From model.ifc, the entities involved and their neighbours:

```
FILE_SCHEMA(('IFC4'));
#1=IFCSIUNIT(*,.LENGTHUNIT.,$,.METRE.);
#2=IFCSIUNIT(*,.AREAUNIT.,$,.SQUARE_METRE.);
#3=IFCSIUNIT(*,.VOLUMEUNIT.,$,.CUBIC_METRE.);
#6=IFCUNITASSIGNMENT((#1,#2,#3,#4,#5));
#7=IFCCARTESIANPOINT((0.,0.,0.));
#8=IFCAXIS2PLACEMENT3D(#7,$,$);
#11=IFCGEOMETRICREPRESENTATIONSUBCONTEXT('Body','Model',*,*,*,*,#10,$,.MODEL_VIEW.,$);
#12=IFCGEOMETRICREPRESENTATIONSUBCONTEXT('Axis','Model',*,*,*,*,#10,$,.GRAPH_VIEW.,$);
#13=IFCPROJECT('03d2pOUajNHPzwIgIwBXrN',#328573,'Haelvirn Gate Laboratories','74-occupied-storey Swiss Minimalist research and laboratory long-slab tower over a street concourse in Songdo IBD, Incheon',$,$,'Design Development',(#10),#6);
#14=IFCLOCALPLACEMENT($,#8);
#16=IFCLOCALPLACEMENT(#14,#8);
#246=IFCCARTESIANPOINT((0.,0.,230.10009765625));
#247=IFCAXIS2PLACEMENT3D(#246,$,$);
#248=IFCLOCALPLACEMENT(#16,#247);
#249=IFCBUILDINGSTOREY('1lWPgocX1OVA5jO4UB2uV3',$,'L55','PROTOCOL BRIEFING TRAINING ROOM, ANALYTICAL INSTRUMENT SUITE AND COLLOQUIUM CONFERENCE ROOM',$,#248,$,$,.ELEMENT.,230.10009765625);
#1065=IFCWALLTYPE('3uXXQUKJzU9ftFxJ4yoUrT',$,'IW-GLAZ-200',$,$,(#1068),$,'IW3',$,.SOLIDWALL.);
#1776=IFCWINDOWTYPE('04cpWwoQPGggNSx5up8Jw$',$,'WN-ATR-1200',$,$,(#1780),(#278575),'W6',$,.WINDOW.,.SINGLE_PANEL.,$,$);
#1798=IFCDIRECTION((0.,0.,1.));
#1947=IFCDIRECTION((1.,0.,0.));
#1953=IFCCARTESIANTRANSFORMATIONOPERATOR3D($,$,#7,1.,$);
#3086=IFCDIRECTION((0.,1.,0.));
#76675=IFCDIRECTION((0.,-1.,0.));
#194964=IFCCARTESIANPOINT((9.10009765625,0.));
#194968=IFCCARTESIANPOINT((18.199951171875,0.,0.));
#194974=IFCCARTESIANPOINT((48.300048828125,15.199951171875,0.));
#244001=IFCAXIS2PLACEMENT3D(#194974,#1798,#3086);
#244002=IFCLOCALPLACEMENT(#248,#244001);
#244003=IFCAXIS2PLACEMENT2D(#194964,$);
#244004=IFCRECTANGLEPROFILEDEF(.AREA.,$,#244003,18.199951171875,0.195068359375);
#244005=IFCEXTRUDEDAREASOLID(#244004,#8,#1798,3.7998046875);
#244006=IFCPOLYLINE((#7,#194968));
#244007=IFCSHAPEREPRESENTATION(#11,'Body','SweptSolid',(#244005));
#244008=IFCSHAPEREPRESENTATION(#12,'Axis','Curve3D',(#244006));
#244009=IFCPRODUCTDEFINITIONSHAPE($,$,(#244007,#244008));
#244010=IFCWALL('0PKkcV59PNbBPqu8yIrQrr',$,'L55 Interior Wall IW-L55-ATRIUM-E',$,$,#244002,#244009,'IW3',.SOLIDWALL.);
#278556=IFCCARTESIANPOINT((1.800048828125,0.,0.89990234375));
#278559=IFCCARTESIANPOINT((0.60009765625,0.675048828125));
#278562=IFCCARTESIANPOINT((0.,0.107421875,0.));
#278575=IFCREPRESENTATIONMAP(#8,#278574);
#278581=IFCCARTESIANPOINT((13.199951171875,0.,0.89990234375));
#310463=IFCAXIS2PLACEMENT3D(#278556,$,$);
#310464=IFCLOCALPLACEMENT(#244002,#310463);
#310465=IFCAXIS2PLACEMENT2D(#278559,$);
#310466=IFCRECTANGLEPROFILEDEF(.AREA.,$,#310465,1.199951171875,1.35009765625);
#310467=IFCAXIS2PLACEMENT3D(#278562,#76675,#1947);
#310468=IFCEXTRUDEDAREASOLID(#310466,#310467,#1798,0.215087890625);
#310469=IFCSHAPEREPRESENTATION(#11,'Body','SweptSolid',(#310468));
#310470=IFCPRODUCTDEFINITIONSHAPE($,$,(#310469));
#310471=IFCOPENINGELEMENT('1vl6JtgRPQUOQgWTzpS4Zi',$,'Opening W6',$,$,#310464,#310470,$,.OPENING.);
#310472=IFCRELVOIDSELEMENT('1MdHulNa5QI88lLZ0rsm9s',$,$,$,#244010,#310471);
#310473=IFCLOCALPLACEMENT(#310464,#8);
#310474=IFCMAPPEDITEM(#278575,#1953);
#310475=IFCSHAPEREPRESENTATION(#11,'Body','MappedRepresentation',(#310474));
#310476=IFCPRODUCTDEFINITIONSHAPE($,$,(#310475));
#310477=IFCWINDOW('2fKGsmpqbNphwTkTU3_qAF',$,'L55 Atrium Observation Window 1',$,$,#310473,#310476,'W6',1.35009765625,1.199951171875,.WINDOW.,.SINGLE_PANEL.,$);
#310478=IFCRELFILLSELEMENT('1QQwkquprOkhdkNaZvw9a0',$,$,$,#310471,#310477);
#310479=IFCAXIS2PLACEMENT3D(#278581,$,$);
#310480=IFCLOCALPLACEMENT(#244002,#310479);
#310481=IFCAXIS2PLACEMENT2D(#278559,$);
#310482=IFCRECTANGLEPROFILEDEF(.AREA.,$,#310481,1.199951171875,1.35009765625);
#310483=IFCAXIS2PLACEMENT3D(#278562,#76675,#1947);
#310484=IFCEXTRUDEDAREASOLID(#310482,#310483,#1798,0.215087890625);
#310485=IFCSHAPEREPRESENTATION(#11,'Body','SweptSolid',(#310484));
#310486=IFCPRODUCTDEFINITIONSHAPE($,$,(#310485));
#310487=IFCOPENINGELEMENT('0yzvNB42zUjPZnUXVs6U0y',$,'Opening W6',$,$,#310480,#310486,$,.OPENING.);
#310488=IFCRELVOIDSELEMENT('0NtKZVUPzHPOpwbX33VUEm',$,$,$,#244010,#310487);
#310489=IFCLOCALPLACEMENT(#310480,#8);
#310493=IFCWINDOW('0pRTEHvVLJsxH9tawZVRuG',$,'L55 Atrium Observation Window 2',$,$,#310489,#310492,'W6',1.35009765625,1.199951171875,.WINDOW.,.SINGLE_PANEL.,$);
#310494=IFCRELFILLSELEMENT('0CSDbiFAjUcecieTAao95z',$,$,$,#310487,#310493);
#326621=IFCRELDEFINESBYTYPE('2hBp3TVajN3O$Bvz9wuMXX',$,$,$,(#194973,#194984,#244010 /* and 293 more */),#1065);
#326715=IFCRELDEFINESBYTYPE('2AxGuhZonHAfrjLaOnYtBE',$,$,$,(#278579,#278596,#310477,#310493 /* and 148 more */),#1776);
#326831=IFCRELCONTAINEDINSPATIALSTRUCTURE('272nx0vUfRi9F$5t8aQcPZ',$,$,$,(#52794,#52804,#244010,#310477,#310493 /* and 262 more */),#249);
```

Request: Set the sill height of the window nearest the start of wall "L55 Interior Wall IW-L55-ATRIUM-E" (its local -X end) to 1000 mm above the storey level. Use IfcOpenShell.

```python
import numpy as np
import ifcopenshell
import ifcopenshell.api.geometry
import ifcopenshell.geom
import ifcopenshell.util.element
import ifcopenshell.util.placement
import ifcopenshell.util.shape
import ifcopenshell.util.unit

model = ifcopenshell.open("model.ifc")
unit_scale = ifcopenshell.util.unit.calculate_unit_scale(model)

window = model.by_guid("2fKGsmpqbNphwTkTU3_qAF")
opening = window.FillsVoids[0].RelatingOpeningElement
storey = ifcopenshell.util.element.get_container(window, ifc_class="IfcBuildingStorey")
level = ifcopenshell.util.placement.get_local_placement(storey.ObjectPlacement)[2, 3]

# The opening's origin need not be at the sill, so measure its lowest point.
shape = ifcopenshell.geom.create_shape(ifcopenshell.geom.settings(), opening)
bottom = ifcopenshell.util.shape.get_shape_bottom_elevation(shape, shape.geometry) / unit_scale
dz = level + 1 / unit_scale - bottom

shift = np.array([0.0, 0.0, dz])
# The window is placed relative to its opening, so it follows when the opening moves.
matrix = ifcopenshell.util.placement.get_local_placement(opening.ObjectPlacement)
matrix[:3, 3] += shift
ifcopenshell.api.geometry.edit_object_placement(
    model, product=opening, matrix=matrix, is_si=False, should_transform_children=True
)

print(f"moved by {dz * unit_scale:+.3f} m")

model.write("model_v2.ifc")
```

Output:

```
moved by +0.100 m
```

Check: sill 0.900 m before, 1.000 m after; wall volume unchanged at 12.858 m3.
